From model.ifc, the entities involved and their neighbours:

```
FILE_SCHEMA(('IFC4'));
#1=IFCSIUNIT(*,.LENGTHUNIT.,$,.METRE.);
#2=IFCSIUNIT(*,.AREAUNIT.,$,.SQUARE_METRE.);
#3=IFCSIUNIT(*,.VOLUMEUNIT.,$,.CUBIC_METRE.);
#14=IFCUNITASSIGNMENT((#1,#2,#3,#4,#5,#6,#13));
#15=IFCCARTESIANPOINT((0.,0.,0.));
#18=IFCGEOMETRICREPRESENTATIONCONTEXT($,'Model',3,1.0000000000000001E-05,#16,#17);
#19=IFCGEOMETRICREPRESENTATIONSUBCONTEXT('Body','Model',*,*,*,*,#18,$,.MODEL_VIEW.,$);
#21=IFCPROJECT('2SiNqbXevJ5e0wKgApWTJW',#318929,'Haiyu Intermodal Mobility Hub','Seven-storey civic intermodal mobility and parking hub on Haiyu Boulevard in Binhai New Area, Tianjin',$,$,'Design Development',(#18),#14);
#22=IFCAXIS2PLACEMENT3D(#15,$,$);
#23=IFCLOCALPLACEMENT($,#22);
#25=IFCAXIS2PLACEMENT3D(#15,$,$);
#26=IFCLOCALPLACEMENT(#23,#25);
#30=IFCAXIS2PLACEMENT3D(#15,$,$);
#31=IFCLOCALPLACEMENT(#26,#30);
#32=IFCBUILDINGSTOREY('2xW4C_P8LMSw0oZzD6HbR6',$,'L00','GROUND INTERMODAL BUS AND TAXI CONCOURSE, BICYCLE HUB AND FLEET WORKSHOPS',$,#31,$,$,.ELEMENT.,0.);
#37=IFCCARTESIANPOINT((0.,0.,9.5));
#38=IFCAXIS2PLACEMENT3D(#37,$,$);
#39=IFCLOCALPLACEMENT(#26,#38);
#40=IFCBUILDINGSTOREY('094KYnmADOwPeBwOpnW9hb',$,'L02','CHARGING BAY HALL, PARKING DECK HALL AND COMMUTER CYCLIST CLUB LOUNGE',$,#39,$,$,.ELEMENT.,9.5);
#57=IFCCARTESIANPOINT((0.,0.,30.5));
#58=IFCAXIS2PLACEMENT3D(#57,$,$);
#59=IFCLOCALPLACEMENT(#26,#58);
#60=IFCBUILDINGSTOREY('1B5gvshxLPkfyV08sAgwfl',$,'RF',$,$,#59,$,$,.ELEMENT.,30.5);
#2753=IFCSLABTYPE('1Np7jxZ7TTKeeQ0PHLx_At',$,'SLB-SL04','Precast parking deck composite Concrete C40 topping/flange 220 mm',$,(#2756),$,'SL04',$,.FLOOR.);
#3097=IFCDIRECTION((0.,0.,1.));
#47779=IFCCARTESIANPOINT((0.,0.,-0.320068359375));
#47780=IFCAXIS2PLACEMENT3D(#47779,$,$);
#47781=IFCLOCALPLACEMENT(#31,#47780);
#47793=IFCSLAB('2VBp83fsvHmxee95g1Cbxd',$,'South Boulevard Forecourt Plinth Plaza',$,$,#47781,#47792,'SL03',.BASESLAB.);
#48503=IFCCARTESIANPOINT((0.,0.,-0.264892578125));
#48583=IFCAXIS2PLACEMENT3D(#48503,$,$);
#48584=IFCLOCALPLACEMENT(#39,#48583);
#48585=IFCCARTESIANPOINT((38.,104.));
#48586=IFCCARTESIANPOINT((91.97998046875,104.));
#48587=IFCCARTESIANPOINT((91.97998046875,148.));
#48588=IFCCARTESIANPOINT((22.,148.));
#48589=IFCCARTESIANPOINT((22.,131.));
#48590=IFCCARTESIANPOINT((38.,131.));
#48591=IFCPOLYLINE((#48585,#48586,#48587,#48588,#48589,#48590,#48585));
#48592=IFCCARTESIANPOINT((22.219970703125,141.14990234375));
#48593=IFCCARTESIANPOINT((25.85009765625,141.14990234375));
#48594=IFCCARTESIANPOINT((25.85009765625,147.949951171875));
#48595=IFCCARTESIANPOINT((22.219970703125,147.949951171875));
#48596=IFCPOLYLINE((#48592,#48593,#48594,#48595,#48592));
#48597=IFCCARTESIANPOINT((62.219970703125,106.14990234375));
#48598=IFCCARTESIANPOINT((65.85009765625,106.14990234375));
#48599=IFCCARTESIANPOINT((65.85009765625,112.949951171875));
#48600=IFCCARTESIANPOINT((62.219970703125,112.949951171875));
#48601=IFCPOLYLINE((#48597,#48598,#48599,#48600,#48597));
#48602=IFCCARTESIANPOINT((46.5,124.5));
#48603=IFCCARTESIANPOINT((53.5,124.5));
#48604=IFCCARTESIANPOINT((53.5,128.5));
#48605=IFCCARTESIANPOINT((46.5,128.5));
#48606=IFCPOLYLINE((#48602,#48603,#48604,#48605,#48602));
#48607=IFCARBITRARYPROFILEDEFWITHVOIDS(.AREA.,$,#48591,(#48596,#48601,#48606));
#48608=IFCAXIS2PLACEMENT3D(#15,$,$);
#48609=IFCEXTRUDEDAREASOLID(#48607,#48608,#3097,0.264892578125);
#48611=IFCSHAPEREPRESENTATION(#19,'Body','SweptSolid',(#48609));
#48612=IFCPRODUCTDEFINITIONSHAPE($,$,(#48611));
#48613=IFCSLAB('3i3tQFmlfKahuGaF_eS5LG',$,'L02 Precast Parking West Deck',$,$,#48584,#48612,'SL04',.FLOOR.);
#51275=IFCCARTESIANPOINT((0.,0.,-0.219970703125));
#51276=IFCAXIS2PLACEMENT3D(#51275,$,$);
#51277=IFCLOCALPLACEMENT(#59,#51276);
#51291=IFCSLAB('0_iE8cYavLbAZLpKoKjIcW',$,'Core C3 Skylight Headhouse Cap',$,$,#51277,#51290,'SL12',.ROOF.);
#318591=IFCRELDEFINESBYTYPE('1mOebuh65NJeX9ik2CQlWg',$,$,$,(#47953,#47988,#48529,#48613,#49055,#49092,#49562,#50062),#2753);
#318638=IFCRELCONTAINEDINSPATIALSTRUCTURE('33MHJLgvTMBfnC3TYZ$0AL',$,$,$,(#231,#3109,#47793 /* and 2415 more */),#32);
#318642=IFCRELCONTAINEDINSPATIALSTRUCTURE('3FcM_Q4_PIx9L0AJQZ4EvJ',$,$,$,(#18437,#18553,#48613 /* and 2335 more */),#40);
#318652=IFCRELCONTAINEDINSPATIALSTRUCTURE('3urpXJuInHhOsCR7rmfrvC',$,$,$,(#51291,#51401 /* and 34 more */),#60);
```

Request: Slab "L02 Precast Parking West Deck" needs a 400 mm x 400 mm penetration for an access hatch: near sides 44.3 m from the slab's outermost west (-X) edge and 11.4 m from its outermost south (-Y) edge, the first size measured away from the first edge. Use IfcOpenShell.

```python
import numpy as np
import ifcopenshell
import ifcopenshell.api.feature
import ifcopenshell.api.geometry
import ifcopenshell.api.root
import ifcopenshell.geom
import ifcopenshell.util.placement
import ifcopenshell.util.representation
import ifcopenshell.util.shape
import ifcopenshell.util.unit

model = ifcopenshell.open("model.ifc")
unit_scale = ifcopenshell.util.unit.calculate_unit_scale(model)
settings = ifcopenshell.geom.settings()


def volume(element):
    """Net volume in cubic metres, openings subtracted."""
    shape = ifcopenshell.geom.create_shape(settings, element)
    return ifcopenshell.util.shape.get_volume(shape.geometry)


slab = model.by_id(48613)
before = volume(slab)

# Extent in the slab's own axes, in metres. The edges named are its -X and -Y sides.
slab_shape = ifcopenshell.geom.create_shape(settings, slab)
vertices = ifcopenshell.util.shape.get_vertices(slab_shape.geometry)
x_min, y_min, bottom = vertices.min(axis=0)
top = vertices[:, 2].max()

opening = ifcopenshell.api.root.create_entity(model, ifc_class="IfcOpeningElement", name="Access hatch opening", predefined_type="OPENING")
context = ifcopenshell.util.representation.get_context(model, "Model", "Body", "MODEL_VIEW")
width, depth = 0.4, 0.4
outline = [(0.0, 0.0), (width, 0.0), (width, depth), (0.0, depth), (0.0, 0.0)]
# Overshoot both faces by 50 mm so the cut is clean.
shape = ifcopenshell.api.geometry.add_slab_representation(
    model, context=context, depth=top - bottom + 0.1, polyline=outline
)
ifcopenshell.api.geometry.assign_representation(model, product=opening, representation=shape)

matrix = ifcopenshell.util.placement.get_local_placement(slab.ObjectPlacement)
matrix[:, 3] = matrix @ np.append(np.array([x_min + 44.3, y_min + 11.4, bottom - 0.05]) / unit_scale, 1.0)
ifcopenshell.api.geometry.edit_object_placement(model, product=opening, matrix=matrix, is_si=False)
ifcopenshell.api.feature.add_feature(model, feature=opening, element=slab)

after = volume(slab)

print(f"slab volume {before:.3f} -> {after:.3f} m3")

model.write("model_edited.ifc")
```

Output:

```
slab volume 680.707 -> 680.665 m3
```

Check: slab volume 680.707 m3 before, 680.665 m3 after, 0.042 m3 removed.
